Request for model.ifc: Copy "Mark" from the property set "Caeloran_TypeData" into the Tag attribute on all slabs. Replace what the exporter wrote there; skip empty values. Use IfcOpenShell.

First a look at what the model holds.

```python
import ifcopenshell
import ifcopenshell.util.element

model = ifcopenshell.open("model.ifc")
print(model.schema)
slabs = model.by_type("IfcSlab")
print(len(slabs), "slabs")
for e in slabs[:8]:
    source = ifcopenshell.util.element.get_pset(e, "Caeloran_TypeData", "Mark")
    target = e.Tag
    print(e.id(), repr(source), repr(target), sep=" | ")
```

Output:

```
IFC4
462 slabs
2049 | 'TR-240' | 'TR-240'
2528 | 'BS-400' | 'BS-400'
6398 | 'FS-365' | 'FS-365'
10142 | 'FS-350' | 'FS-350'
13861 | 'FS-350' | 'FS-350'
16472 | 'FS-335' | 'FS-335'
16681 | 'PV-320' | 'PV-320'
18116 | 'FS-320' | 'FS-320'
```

```python
import ifcopenshell
import ifcopenshell.util.element

model = ifcopenshell.open("model.ifc")

count = 0
for e in model.by_type("IfcSlab"):
    value = ifcopenshell.util.element.get_pset(e, "Caeloran_TypeData", "Mark")
    current = e.Tag
    if not value or not value.strip() or current == value:
        continue
    e.Tag = value
    count += 1

print(count, "slabs updated")

model.write("model-out.ifc")
```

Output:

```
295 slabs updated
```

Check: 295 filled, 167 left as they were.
